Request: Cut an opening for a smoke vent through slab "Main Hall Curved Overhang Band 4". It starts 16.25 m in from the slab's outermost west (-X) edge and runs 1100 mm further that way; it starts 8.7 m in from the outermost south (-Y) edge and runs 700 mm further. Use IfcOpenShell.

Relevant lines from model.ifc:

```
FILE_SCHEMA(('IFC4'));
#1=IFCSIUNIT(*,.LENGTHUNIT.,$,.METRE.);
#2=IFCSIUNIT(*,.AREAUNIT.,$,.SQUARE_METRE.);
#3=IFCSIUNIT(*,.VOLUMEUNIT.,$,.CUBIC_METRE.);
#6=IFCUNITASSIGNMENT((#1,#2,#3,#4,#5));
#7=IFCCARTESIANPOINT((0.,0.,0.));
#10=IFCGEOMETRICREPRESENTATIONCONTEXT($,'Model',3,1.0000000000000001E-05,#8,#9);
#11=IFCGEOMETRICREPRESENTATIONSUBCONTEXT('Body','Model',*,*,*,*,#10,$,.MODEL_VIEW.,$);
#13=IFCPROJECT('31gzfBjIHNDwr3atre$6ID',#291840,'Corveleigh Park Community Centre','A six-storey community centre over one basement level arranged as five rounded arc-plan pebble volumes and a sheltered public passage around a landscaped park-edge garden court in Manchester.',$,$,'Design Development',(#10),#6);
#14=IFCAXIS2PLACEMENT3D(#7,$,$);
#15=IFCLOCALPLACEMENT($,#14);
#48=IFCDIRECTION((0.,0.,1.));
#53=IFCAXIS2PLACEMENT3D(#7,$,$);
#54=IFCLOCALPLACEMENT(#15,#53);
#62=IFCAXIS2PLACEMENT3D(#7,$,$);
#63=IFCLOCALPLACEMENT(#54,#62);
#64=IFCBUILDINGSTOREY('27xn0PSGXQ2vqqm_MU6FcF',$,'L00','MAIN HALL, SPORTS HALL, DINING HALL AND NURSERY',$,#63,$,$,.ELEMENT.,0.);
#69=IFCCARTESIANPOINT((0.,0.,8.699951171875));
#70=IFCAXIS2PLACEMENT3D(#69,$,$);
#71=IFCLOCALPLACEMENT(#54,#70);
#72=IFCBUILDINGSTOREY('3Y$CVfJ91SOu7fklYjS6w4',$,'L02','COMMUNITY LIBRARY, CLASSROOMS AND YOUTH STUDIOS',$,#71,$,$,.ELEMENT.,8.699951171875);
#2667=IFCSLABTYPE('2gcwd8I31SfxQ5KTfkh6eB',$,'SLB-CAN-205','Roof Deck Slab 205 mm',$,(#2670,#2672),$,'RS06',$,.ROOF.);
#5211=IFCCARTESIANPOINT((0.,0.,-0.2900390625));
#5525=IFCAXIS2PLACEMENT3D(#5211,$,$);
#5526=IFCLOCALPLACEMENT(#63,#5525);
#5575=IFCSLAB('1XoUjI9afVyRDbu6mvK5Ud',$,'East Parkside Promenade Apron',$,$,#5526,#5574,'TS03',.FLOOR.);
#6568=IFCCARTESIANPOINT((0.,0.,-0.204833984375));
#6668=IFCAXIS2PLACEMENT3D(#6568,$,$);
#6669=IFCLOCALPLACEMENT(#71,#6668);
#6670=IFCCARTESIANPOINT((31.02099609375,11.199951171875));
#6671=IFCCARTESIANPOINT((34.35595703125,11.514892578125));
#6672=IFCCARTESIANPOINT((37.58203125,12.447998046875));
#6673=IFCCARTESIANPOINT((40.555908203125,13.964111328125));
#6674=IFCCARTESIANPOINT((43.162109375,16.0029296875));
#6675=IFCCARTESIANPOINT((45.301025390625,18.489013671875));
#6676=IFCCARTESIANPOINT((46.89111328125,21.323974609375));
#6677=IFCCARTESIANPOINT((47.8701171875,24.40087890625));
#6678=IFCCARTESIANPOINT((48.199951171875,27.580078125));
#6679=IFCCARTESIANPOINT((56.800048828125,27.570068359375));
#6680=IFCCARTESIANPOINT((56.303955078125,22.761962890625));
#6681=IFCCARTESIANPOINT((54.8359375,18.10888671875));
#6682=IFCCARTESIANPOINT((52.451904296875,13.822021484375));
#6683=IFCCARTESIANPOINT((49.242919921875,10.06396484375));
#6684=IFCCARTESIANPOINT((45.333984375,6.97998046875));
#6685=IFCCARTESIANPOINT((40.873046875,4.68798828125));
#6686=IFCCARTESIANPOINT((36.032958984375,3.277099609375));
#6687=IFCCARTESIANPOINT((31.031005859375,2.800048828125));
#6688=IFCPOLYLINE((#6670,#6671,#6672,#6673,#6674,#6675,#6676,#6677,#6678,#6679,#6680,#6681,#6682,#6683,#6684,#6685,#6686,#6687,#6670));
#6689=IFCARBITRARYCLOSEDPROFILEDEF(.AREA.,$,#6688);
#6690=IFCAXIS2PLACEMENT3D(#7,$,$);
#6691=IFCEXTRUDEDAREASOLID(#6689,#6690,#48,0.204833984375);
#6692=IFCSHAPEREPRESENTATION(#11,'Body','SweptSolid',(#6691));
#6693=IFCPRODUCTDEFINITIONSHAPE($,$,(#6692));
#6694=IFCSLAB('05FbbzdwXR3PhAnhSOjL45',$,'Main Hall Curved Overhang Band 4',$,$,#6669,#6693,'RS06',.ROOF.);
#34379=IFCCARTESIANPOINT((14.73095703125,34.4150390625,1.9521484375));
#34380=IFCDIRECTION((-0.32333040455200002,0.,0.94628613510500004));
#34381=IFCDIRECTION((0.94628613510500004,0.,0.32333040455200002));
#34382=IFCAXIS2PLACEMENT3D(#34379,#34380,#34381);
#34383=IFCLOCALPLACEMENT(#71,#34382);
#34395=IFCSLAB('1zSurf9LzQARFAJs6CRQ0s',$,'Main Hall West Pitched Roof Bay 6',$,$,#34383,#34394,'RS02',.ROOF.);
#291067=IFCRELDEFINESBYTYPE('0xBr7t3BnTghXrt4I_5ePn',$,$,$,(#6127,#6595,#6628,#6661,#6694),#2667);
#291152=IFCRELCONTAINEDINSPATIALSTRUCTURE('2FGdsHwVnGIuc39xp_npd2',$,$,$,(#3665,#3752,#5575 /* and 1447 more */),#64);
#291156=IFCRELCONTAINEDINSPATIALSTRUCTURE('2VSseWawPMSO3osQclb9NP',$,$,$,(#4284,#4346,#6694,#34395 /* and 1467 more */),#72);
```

```python
import numpy as np
import ifcopenshell
import ifcopenshell.api.feature
import ifcopenshell.api.geometry
import ifcopenshell.api.root
import ifcopenshell.geom
import ifcopenshell.util.placement
import ifcopenshell.util.representation
import ifcopenshell.util.shape
import ifcopenshell.util.unit

model = ifcopenshell.open("model.ifc")
unit_scale = ifcopenshell.util.unit.calculate_unit_scale(model)
settings = ifcopenshell.geom.settings()


def volume(element):
    """Net volume in cubic metres, openings subtracted."""
    shape = ifcopenshell.geom.create_shape(settings, element)
    return ifcopenshell.util.shape.get_volume(shape.geometry)


slab = model.by_id(6694)
before = volume(slab)

# Extent in the slab's own axes, in metres. The edges named are its -X and -Y sides.
slab_shape = ifcopenshell.geom.create_shape(settings, slab)
vertices = ifcopenshell.util.shape.get_vertices(slab_shape.geometry)
x_min, y_min, bottom = vertices.min(axis=0)
top = vertices[:, 2].max()

opening = ifcopenshell.api.root.create_entity(model, ifc_class="IfcOpeningElement", name="Smoke vent opening", predefined_type="OPENING")
context = ifcopenshell.util.representation.get_context(model, "Model", "Body", "MODEL_VIEW")
width, depth = 1.1, 0.7
outline = [(0.0, 0.0), (width, 0.0), (width, depth), (0.0, depth), (0.0, 0.0)]
# Overshoot both faces by 50 mm so the cut is clean.
shape = ifcopenshell.api.geometry.add_slab_representation(
    model, context=context, depth=top - bottom + 0.1, polyline=outline
)
ifcopenshell.api.geometry.assign_representation(model, product=opening, representation=shape)

matrix = ifcopenshell.util.placement.get_local_placement(slab.ObjectPlacement)
matrix[:, 3] = matrix @ np.append(np.array([x_min + 16.25, y_min + 8.7, bottom - 0.05]) / unit_scale, 1.0)
ifcopenshell.api.geometry.edit_object_placement(model, product=opening, matrix=matrix, is_si=False)
ifcopenshell.api.feature.add_feature(model, feature=opening, element=slab)

after = volume(slab)

print(f"slab volume {before:.3f} -> {after:.3f} m3")

model.write("model_rev.ifc")
```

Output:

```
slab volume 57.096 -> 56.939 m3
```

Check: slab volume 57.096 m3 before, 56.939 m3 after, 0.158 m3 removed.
